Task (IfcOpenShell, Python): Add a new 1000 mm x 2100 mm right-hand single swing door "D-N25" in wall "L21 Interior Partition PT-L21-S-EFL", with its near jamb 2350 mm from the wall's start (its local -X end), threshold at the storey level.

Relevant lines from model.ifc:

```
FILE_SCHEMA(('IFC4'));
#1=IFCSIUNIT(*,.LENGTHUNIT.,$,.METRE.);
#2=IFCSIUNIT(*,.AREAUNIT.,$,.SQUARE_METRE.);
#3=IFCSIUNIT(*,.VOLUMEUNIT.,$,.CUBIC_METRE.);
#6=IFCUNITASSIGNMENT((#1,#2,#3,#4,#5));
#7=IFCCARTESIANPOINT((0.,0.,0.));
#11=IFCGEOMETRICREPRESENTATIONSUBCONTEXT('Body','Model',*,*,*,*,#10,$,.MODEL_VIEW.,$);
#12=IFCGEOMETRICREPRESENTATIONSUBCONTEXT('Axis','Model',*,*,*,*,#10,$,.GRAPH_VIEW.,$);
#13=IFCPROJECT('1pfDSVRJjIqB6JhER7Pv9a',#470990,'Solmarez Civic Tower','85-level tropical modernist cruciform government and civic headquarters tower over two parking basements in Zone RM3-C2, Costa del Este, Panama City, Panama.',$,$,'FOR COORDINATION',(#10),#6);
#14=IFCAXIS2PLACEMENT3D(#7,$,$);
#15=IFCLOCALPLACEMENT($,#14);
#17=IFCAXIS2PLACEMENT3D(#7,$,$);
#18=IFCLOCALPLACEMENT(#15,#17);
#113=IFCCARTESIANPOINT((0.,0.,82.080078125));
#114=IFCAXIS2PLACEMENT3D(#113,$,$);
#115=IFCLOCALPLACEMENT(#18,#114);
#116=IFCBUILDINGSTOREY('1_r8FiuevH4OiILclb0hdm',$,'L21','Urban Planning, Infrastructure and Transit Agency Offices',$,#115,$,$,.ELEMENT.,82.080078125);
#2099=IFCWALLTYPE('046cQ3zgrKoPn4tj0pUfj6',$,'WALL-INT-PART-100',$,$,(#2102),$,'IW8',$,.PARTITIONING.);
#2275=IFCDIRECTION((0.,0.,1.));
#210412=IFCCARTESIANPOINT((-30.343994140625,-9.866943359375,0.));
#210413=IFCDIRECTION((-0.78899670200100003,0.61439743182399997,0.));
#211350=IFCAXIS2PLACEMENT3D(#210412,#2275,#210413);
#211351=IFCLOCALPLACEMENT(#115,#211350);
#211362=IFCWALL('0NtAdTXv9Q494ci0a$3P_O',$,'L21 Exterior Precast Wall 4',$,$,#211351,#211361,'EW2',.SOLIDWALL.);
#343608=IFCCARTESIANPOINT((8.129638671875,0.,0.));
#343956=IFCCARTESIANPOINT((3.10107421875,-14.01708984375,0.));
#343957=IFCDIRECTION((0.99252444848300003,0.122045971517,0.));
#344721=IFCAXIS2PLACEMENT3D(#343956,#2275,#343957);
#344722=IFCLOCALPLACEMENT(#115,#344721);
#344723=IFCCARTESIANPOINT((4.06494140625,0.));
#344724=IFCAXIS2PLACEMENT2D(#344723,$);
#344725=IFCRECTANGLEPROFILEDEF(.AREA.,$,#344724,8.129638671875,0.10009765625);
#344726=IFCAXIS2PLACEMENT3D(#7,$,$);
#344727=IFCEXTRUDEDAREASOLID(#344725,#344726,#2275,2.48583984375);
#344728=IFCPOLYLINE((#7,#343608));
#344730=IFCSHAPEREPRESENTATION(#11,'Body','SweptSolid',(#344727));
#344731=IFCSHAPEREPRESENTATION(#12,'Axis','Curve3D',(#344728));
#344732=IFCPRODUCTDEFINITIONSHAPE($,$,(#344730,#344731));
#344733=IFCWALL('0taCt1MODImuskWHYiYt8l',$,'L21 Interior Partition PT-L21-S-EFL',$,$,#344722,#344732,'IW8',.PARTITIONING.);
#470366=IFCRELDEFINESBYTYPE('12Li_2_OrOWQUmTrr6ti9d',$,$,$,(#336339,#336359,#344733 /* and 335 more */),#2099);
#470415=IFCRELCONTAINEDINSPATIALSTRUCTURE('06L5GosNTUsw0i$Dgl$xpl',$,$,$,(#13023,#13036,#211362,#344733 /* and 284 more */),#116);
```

```python
import numpy as np
import ifcopenshell
import ifcopenshell.api.feature
import ifcopenshell.api.geometry
import ifcopenshell.api.root
import ifcopenshell.api.spatial
import ifcopenshell.geom
import ifcopenshell.util.element
import ifcopenshell.util.placement
import ifcopenshell.util.representation
import ifcopenshell.util.shape
import ifcopenshell.util.unit

model = ifcopenshell.open("model.ifc")
unit_scale = ifcopenshell.util.unit.calculate_unit_scale(model)
settings = ifcopenshell.geom.settings()


def volume(element):
    """Net volume in cubic metres, openings subtracted."""
    shape = ifcopenshell.geom.create_shape(settings, element)
    return ifcopenshell.util.shape.get_volume(shape.geometry)


wall = model.by_guid("0taCt1MODImuskWHYiYt8l")
storey = ifcopenshell.util.element.get_container(wall, ifc_class="IfcBuildingStorey")
context = ifcopenshell.util.representation.get_context(model, "Model", "Body", "MODEL_VIEW")
before = volume(wall)

width, height, from_end, sill = 1, 2.1, 2.35, 0.0  # metres

# The wall runs along its own X axis, and the end named is its -X end.
wall_shape = ifcopenshell.geom.create_shape(settings, wall)
x, y, z = ifcopenshell.util.shape.get_vertices(wall_shape.geometry).T
start = x.min() + from_end
face, thickness = float(y.min()), float(y.max() - y.min())
wall_matrix = ifcopenshell.util.placement.get_local_placement(wall.ObjectPlacement)
level = ifcopenshell.util.placement.get_local_placement(storey.ObjectPlacement)[2, 3]


def in_wall(x, y):
    """Placement at x, y metres in the wall's axes, at sill height."""
    matrix = wall_matrix.copy()
    matrix[:, 3] = wall_matrix @ np.array([x / unit_scale, y / unit_scale, 0.0, 1.0])
    matrix[2, 3] = level + sill / unit_scale
    return matrix


# Opening: a box that overshoots both wall faces by 50 mm.
opening = ifcopenshell.api.root.create_entity(model, ifc_class="IfcOpeningElement", predefined_type="OPENING")
box = ifcopenshell.api.geometry.add_wall_representation(
    model, context=context, length=width, height=height, thickness=thickness + 0.1
)
ifcopenshell.api.geometry.assign_representation(model, product=opening, representation=box)
ifcopenshell.api.geometry.edit_object_placement(model, product=opening, matrix=in_wall(start, face - 0.05), is_si=False)
ifcopenshell.api.feature.add_feature(model, feature=opening, element=wall)

door = ifcopenshell.api.root.create_entity(model, ifc_class="IfcDoor", name="D-N25", predefined_type="DOOR")
door.OverallWidth, door.OverallHeight = width / unit_scale, height / unit_scale
door.OperationType = "SINGLE_SWING_RIGHT"
body = ifcopenshell.api.geometry.add_door_representation(
    model,
    context=context,
    overall_width=door.OverallWidth,
    overall_height=door.OverallHeight,
    operation_type="SINGLE_SWING_RIGHT",
    lining_properties={"LiningDepth": thickness / unit_scale, "ThresholdDepth": thickness / unit_scale},
)
ifcopenshell.api.geometry.assign_representation(model, product=door, representation=body)
ifcopenshell.api.spatial.assign_container(model, products=[door], relating_structure=storey)
ifcopenshell.api.feature.add_filling(model, opening=opening, element=door)

# The lining spans the wall, so the door starts at the wall face.
ifcopenshell.api.geometry.edit_object_placement(model, product=door, matrix=in_wall(start, face), is_si=False)

after = volume(wall)

print(f"wall volume {before:.3f} -> {after:.3f} m3")

model.write("model_v2.ifc")
```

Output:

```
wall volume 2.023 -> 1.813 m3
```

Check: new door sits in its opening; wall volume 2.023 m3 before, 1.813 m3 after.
